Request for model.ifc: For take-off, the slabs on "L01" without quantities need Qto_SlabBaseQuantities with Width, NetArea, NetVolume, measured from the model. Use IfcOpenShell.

First a look at what the model holds.

```python
import ifcopenshell
import ifcopenshell.util.element
import ifcopenshell.util.unit

model = ifcopenshell.open("model.ifc")
print(model.schema)
for unit_type in ("LENGTHUNIT", "AREAUNIT", "VOLUMEUNIT"):
    print(unit_type, ifcopenshell.util.unit.calculate_unit_scale(model, unit_type))
storey = next(s for s in model.by_type("IfcBuildingStorey") if s.Name == "L01")
slabs = [e for e in ifcopenshell.util.element.get_decomposition(storey) if e.is_a("IfcSlab")]
for e in sorted(slabs, key=lambda e: e.id()):
    print(e.id(), e.is_a(), e.Name, list(ifcopenshell.util.element.get_psets(e, qtos_only=True)), sep=" | ")
```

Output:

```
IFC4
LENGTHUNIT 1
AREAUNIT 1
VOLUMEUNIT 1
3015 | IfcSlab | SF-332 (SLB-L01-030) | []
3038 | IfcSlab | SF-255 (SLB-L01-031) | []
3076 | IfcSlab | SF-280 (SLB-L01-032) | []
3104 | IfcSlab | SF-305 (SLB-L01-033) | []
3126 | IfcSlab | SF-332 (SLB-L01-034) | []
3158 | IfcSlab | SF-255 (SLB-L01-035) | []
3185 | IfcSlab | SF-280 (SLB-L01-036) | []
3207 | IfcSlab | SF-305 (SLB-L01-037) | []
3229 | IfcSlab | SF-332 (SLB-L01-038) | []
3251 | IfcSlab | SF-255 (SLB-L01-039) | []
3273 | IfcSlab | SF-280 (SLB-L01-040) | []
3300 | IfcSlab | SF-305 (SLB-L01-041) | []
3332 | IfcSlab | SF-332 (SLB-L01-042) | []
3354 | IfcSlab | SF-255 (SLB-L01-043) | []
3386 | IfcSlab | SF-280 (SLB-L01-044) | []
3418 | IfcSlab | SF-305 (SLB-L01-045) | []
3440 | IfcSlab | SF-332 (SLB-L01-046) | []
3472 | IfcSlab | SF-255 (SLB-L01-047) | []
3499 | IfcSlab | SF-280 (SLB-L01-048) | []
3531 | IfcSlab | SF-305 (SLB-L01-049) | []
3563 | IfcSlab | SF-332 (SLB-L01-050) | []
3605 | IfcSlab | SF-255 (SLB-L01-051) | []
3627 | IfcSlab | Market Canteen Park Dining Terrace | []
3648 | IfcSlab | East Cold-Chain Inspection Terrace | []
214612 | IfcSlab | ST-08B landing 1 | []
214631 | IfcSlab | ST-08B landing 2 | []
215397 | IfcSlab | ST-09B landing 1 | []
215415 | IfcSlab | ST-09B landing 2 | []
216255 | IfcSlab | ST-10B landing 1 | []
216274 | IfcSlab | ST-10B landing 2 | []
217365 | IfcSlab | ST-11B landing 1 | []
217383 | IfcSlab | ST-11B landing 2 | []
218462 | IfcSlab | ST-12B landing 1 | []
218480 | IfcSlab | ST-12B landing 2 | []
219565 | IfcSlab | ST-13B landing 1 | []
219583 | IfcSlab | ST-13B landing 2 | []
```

```python
import ifcopenshell
import ifcopenshell.api.pset
import ifcopenshell.geom
import ifcopenshell.util.element
import ifcopenshell.util.shape
import ifcopenshell.util.unit

model = ifcopenshell.open("model.ifc")
unit_scale = ifcopenshell.util.unit.calculate_unit_scale(model)
area_scale = ifcopenshell.util.unit.calculate_unit_scale(model, "AREAUNIT")
volume_scale = ifcopenshell.util.unit.calculate_unit_scale(model, "VOLUMEUNIT")
settings = ifcopenshell.geom.settings()

storey = next(s for s in model.by_type("IfcBuildingStorey") if s.Name == "L01")
slabs = [e for e in ifcopenshell.util.element.get_decomposition(storey) if e.is_a("IfcSlab")]

for e in sorted(slabs, key=lambda e: e.id()):
    if ifcopenshell.util.element.get_psets(e, qtos_only=True, should_inherit=False):
        continue
    # Geometry comes back in metres, in the element's own axes.
    shape = ifcopenshell.geom.create_shape(settings, e)
    values = {
        "Width": ifcopenshell.util.shape.get_z(shape.geometry) / unit_scale,
        "NetArea": ifcopenshell.util.shape.get_footprint_area(shape.geometry) / area_scale,
        "NetVolume": ifcopenshell.util.shape.get_volume(shape.geometry) / volume_scale,
    }
    qto = ifcopenshell.api.pset.add_qto(model, product=e, name="Qto_SlabBaseQuantities")
    ifcopenshell.api.pset.edit_qto(model, qto=qto, properties=values)
    print(e.id(), {k: round(v, 3) for k, v in values.items()})

model.write("model-out.ifc")
```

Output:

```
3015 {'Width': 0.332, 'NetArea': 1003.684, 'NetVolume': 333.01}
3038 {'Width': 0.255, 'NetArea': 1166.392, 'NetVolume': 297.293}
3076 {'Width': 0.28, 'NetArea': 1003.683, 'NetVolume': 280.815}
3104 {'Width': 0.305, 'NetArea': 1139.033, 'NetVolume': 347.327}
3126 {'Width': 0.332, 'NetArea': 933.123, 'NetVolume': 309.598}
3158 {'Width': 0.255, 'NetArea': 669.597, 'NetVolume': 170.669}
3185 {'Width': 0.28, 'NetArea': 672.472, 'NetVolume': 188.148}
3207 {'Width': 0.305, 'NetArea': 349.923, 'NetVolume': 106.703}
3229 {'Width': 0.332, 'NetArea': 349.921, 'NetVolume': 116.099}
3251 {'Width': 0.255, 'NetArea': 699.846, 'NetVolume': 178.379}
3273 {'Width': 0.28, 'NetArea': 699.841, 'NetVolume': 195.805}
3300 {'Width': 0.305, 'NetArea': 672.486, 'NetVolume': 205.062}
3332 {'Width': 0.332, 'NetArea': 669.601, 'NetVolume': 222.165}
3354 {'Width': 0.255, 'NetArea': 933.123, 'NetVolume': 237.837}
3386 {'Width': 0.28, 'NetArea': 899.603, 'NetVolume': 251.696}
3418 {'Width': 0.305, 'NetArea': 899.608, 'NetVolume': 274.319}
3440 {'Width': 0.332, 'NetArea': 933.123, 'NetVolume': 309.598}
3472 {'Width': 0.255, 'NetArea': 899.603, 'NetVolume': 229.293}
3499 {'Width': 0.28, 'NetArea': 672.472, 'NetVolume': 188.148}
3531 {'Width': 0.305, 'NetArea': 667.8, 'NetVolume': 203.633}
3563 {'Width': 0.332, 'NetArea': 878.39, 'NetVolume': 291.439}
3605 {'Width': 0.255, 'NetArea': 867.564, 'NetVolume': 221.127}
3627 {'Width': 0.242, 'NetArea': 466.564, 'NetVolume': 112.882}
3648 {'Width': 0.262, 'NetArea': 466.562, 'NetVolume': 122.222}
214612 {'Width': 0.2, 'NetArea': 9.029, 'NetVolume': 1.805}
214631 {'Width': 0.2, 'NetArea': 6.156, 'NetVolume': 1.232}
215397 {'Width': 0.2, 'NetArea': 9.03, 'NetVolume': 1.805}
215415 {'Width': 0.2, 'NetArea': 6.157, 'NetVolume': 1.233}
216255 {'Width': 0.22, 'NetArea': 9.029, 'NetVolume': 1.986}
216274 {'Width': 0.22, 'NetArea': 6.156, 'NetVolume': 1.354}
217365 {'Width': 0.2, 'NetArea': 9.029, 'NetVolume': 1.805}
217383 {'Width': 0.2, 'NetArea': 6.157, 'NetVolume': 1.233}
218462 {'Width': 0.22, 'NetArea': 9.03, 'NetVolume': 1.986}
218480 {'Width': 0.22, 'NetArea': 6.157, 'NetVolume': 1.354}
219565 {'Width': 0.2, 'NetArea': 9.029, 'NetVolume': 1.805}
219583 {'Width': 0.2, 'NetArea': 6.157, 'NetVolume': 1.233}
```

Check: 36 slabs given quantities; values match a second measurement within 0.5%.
